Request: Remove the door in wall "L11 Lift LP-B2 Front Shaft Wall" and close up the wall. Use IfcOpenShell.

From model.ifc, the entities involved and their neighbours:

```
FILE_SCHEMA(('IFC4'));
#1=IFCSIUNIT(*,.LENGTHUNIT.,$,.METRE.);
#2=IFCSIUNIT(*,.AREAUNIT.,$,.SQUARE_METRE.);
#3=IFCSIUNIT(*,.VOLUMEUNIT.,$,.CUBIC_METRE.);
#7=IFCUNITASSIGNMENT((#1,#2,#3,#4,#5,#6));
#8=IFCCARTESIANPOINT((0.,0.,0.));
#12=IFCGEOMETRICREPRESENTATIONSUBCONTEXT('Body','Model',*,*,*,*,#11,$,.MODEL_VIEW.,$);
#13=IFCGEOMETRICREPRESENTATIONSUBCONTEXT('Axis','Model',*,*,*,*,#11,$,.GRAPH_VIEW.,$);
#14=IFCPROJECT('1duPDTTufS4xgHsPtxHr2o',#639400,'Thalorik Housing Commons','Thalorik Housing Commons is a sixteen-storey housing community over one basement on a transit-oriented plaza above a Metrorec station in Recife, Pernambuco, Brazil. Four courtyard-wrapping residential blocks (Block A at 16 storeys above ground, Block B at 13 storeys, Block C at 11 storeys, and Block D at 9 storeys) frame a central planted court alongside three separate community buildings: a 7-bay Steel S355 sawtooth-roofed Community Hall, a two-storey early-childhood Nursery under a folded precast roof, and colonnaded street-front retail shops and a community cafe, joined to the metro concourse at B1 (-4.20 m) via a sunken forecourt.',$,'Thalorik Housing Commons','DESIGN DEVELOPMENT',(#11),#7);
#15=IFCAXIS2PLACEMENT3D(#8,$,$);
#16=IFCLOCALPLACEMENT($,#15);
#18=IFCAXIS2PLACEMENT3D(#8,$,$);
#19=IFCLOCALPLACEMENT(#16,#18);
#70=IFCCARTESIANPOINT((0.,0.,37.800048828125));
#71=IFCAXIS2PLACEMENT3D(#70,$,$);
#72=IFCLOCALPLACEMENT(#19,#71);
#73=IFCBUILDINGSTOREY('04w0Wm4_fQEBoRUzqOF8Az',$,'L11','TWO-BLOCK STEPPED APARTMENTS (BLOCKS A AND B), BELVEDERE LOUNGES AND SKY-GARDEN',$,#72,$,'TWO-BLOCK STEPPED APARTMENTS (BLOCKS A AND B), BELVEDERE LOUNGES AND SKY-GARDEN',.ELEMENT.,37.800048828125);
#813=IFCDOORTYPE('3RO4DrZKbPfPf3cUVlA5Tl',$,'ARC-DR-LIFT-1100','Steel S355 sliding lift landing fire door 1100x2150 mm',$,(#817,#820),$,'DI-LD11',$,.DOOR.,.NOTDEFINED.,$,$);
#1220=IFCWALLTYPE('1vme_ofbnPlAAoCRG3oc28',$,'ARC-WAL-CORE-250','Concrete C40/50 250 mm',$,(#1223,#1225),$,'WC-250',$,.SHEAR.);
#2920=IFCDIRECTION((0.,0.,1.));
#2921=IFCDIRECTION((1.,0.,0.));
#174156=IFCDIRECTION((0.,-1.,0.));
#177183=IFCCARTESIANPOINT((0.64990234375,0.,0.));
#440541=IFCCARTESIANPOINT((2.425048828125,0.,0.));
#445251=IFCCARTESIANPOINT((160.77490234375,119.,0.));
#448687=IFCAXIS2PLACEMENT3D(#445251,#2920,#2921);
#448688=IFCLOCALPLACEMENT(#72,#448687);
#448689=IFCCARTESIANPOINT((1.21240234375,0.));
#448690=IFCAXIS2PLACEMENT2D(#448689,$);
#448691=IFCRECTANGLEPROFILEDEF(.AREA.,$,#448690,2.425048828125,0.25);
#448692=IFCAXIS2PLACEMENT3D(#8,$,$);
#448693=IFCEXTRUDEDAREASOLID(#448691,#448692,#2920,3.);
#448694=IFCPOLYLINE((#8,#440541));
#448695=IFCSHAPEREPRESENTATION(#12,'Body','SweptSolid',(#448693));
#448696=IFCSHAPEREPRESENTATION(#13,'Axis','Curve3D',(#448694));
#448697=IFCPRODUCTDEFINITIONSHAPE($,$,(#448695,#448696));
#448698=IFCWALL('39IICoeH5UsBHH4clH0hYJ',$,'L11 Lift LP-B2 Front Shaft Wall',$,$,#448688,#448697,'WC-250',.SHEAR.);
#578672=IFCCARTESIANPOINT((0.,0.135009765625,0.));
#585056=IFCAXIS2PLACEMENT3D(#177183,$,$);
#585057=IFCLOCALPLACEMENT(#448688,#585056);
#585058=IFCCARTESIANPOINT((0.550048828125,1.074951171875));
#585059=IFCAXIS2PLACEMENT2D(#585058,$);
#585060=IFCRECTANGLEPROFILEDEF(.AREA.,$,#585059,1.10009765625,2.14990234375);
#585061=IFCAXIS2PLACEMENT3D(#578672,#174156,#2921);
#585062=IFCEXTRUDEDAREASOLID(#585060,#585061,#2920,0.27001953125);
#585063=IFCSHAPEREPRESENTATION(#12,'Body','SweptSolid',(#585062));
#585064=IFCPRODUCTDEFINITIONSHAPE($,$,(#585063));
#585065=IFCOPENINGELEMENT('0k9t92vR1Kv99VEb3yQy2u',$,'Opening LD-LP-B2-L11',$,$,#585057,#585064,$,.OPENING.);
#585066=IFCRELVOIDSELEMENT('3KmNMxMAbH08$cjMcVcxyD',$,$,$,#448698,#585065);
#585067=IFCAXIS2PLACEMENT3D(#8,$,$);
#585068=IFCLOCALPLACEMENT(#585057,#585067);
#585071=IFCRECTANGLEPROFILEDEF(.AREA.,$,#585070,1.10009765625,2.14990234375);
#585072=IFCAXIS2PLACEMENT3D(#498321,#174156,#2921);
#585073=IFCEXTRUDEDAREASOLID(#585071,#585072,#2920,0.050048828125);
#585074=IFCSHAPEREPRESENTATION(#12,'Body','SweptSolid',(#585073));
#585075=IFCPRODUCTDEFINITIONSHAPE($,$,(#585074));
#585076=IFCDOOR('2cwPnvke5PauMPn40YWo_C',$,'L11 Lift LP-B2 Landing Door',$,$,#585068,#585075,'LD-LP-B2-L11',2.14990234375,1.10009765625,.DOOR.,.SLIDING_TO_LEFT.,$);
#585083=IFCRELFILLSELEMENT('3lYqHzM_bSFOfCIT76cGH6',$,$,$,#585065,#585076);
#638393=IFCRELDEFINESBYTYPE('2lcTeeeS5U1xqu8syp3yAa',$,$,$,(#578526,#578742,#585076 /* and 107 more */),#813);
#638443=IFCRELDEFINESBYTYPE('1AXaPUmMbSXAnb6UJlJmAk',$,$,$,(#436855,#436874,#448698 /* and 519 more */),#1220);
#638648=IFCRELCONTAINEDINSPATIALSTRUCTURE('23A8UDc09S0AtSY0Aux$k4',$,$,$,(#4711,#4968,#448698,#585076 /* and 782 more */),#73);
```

```python
import ifcopenshell
import ifcopenshell.api.feature
import ifcopenshell.api.root
import ifcopenshell.geom
import ifcopenshell.util.shape

model = ifcopenshell.open("model.ifc")
settings = ifcopenshell.geom.settings()


def volume(element):
    """Net volume in cubic metres, openings subtracted."""
    shape = ifcopenshell.geom.create_shape(settings, element)
    return ifcopenshell.util.shape.get_volume(shape.geometry)


door = model.by_guid("2cwPnvke5PauMPn40YWo_C")
opening = door.FillsVoids[0].RelatingOpeningElement
wall = opening.VoidsElements[0].RelatingBuildingElement
before = volume(wall)

ifcopenshell.api.root.remove_product(model, product=door)
ifcopenshell.api.feature.remove_feature(model, feature=opening)

after = volume(wall)

print(f"wall volume {before:.3f} -> {after:.3f} m3")

model.write("model_v2.ifc")
```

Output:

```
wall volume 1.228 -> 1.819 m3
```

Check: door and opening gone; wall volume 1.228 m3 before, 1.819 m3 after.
